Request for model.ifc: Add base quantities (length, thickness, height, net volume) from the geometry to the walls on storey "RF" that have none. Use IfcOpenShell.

First a look at what the model holds.

```python
import ifcopenshell
import ifcopenshell.util.element
import ifcopenshell.util.unit

model = ifcopenshell.open("model.ifc")
print(model.schema)
for unit_type in ("LENGTHUNIT", "AREAUNIT", "VOLUMEUNIT"):
    print(unit_type, ifcopenshell.util.unit.calculate_unit_scale(model, unit_type))
storey = next(s for s in model.by_type("IfcBuildingStorey") if s.Name == "RF")
walls = [e for e in ifcopenshell.util.element.get_decomposition(storey) if e.is_a("IfcWall")]
for e in sorted(walls, key=lambda e: e.id()):
    print(e.id(), e.is_a(), e.Name, list(ifcopenshell.util.element.get_psets(e, qtos_only=True)), sep=" | ")
```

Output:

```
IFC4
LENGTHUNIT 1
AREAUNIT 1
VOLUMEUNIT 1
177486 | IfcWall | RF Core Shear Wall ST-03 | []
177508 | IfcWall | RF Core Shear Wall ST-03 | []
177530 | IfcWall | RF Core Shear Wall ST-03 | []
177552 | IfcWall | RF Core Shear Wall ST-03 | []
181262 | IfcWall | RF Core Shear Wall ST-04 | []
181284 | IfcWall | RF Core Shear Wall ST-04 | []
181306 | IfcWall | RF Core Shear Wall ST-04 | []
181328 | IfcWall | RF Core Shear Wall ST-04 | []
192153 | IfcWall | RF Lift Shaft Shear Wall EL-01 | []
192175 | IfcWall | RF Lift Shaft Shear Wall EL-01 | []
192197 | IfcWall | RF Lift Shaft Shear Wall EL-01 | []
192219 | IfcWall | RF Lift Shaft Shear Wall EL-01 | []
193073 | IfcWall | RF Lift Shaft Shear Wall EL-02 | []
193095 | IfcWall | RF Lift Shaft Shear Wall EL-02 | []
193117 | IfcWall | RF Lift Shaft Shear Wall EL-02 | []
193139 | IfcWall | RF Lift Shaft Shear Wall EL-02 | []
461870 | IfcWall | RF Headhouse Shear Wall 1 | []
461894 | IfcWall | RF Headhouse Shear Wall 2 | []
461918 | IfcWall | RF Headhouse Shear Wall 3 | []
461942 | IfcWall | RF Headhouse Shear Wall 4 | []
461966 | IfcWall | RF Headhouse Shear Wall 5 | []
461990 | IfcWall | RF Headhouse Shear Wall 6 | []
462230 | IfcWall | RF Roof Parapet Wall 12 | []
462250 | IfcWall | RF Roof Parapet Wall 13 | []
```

```python
import ifcopenshell
import ifcopenshell.api.pset
import ifcopenshell.geom
import ifcopenshell.util.element
import ifcopenshell.util.shape
import ifcopenshell.util.unit

model = ifcopenshell.open("model.ifc")
unit_scale = ifcopenshell.util.unit.calculate_unit_scale(model)
volume_scale = ifcopenshell.util.unit.calculate_unit_scale(model, "VOLUMEUNIT")
settings = ifcopenshell.geom.settings()

storey = next(s for s in model.by_type("IfcBuildingStorey") if s.Name == "RF")
walls = [e for e in ifcopenshell.util.element.get_decomposition(storey) if e.is_a("IfcWall")]

for e in sorted(walls, key=lambda e: e.id()):
    if ifcopenshell.util.element.get_psets(e, qtos_only=True, should_inherit=False):
        continue
    # Geometry comes back in metres, in the element's own axes.
    shape = ifcopenshell.geom.create_shape(settings, e)
    values = {
        "Length": ifcopenshell.util.shape.get_x(shape.geometry) / unit_scale,
        "Width": ifcopenshell.util.shape.get_y(shape.geometry) / unit_scale,
        "Height": ifcopenshell.util.shape.get_z(shape.geometry) / unit_scale,
        "NetVolume": ifcopenshell.util.shape.get_volume(shape.geometry) / volume_scale,
    }
    qto = ifcopenshell.api.pset.add_qto(model, product=e, name="Qto_WallBaseQuantities")
    ifcopenshell.api.pset.edit_qto(model, qto=qto, properties=values)
    print(e.id(), {k: round(v, 3) for k, v in values.items()})

model.write("model_edited.ifc")
```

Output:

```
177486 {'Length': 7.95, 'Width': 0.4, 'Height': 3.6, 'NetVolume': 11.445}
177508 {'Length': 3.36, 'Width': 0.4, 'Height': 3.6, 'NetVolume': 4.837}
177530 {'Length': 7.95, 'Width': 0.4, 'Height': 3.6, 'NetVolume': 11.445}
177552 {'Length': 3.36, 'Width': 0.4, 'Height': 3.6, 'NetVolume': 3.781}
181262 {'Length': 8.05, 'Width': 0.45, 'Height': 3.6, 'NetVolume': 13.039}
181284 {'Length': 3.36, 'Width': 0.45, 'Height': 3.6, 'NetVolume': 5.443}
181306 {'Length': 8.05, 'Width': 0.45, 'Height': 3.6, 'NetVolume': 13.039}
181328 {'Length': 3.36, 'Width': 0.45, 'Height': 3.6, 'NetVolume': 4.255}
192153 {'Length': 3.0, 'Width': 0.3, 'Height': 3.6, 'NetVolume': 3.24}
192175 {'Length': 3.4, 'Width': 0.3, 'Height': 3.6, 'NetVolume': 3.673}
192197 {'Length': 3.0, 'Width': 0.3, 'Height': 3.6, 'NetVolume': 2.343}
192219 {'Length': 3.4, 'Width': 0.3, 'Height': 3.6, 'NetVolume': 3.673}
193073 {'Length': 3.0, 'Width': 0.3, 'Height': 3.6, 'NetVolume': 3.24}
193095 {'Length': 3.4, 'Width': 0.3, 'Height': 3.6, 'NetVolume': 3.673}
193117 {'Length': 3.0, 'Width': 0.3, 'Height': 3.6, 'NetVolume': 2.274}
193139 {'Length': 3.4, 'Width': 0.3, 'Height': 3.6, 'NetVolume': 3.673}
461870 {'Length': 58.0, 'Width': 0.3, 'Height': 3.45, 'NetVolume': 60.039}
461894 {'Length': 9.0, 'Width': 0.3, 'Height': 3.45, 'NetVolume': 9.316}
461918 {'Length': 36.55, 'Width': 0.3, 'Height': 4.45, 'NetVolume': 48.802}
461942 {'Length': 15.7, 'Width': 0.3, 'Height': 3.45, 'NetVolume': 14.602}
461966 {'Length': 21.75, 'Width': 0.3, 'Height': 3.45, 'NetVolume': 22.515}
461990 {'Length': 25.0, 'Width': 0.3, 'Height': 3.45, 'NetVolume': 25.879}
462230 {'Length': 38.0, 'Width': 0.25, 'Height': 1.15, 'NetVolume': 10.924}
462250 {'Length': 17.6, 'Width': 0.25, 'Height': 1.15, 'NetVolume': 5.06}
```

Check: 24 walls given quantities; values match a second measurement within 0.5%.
